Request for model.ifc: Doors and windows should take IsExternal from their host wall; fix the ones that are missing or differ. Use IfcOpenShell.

First a look at what the model holds.

```python
import ifcopenshell
import ifcopenshell.util.element

model = ifcopenshell.open("model.ifc")
print(model.schema)
seen = {}
for e in model.by_type("IfcDoor") + model.by_type("IfcWindow"):
    if not e.FillsVoids:
        continue
    host = e.FillsVoids[0].RelatingOpeningElement.VoidsElements[0].RelatingBuildingElement
    own = ifcopenshell.util.element.get_pset(e, f"Pset_{e.is_a()[3:].removesuffix('StandardCase')}Common", "IsExternal")
    wall = ifcopenshell.util.element.get_pset(host, "Pset_WallCommon", "IsExternal")
    seen[e.is_a(), own, wall] = seen.get((e.is_a(), own, wall), 0) + 1
for (cls, own, wall), count in sorted(seen.items(), key=str):
    print(count, cls, "IsExternal:", own, "| host wall:", wall)
```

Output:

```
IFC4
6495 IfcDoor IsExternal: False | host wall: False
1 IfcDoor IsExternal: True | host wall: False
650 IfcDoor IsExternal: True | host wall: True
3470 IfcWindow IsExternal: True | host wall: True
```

```python
import ifcopenshell
import ifcopenshell.api.pset
import ifcopenshell.util.element

model = ifcopenshell.open("model.ifc")

count = 0
for ifc_class, pset_name in (("IfcDoor", "Pset_DoorCommon"), ("IfcWindow", "Pset_WindowCommon")):
    for e in model.by_type(ifc_class):
        if not e.FillsVoids:
            continue
        host = e.FillsVoids[0].RelatingOpeningElement.VoidsElements[0].RelatingBuildingElement
        external = ifcopenshell.util.element.get_pset(host, "Pset_WallCommon", "IsExternal")
        if external is None or ifcopenshell.util.element.get_pset(e, pset_name, "IsExternal") == external:
            continue
        pset = ifcopenshell.api.pset.add_pset(model, product=e, name=pset_name)
        ifcopenshell.api.pset.edit_pset(model, pset=pset, properties={"IsExternal": external})
        count += 1

print(count, "updated")

model.write("model_updated.ifc")
```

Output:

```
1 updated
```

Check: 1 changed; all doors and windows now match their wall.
